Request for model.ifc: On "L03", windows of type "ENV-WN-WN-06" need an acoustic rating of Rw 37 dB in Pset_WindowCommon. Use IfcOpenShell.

First a look at what the model holds.

```python
import ifcopenshell
import ifcopenshell.util.element

model = ifcopenshell.open("model.ifc")
print(model.schema)
storey = next(s for s in model.by_type("IfcBuildingStorey") if s.Name == "L03")
windows = [e for e in ifcopenshell.util.element.get_decomposition(storey) if e.is_a("IfcWindow")]
seen = {}
for e in windows:
    element_type = ifcopenshell.util.element.get_type(e)
    key = (element_type.Name if element_type != e and element_type else None, ifcopenshell.util.element.get_pset(e, "Pset_WindowCommon", "AcousticRating"))
    seen[key] = seen.get(key, 0) + 1
for (name, value), count in sorted(seen.items(), key=str):
    print(count, "x", name, "|", value)
```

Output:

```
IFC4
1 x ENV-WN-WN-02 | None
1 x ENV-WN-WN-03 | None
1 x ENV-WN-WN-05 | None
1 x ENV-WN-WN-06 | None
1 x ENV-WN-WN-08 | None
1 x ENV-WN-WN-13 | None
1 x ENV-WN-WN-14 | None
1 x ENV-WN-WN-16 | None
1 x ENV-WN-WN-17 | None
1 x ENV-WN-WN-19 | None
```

```python
import ifcopenshell
import ifcopenshell.api.pset
import ifcopenshell.util.element

model = ifcopenshell.open("model.ifc")

storey = next(s for s in model.by_type("IfcBuildingStorey") if s.Name == "L03")
windows = [e for e in ifcopenshell.util.element.get_decomposition(storey) if e.is_a("IfcWindow")]

count = 0
for e in windows:
    element_type = ifcopenshell.util.element.get_type(e)
    if element_type in (None, e) or element_type.Name != "ENV-WN-WN-06":
        continue
    # add_pset returns the element's existing set when there is one.
    pset = ifcopenshell.api.pset.add_pset(model, product=e, name="Pset_WindowCommon")
    ifcopenshell.api.pset.edit_pset(model, pset=pset, properties={"AcousticRating": "Rw 37 dB"})
    count += 1

print(count, "windows updated")

model.write("model_edited.ifc")
```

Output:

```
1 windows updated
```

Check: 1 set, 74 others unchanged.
